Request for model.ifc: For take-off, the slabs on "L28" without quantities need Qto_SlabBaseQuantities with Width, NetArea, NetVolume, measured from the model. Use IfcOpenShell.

First a look at what the model holds.

```python
import ifcopenshell
import ifcopenshell.util.element
import ifcopenshell.util.unit

model = ifcopenshell.open("model.ifc")
print(model.schema)
for unit_type in ("LENGTHUNIT", "AREAUNIT", "VOLUMEUNIT"):
    print(unit_type, ifcopenshell.util.unit.calculate_unit_scale(model, unit_type))
storey = next(s for s in model.by_type("IfcBuildingStorey") if s.Name == "L28")
slabs = [e for e in ifcopenshell.util.element.get_decomposition(storey) if e.is_a("IfcSlab")]
for e in sorted(slabs, key=lambda e: e.id()):
    print(e.id(), e.is_a(), e.Name, list(ifcopenshell.util.element.get_psets(e, qtos_only=True)), sep=" | ")
```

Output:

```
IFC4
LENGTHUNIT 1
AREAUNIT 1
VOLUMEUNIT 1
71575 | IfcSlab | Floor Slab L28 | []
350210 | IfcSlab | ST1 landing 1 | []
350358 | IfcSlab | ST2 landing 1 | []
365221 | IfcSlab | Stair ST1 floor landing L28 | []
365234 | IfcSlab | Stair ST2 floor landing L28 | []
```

```python
import ifcopenshell
import ifcopenshell.api.pset
import ifcopenshell.geom
import ifcopenshell.util.element
import ifcopenshell.util.shape
import ifcopenshell.util.unit

model = ifcopenshell.open("model.ifc")
unit_scale = ifcopenshell.util.unit.calculate_unit_scale(model)
area_scale = ifcopenshell.util.unit.calculate_unit_scale(model, "AREAUNIT")
volume_scale = ifcopenshell.util.unit.calculate_unit_scale(model, "VOLUMEUNIT")
settings = ifcopenshell.geom.settings()

storey = next(s for s in model.by_type("IfcBuildingStorey") if s.Name == "L28")
slabs = [e for e in ifcopenshell.util.element.get_decomposition(storey) if e.is_a("IfcSlab")]

for e in sorted(slabs, key=lambda e: e.id()):
    if ifcopenshell.util.element.get_psets(e, qtos_only=True, should_inherit=False):
        continue
    # Geometry comes back in metres, in the element's own axes.
    shape = ifcopenshell.geom.create_shape(settings, e)
    values = {
        "Width": ifcopenshell.util.shape.get_z(shape.geometry) / unit_scale,
        "NetArea": ifcopenshell.util.shape.get_footprint_area(shape.geometry) / area_scale,
        "NetVolume": ifcopenshell.util.shape.get_volume(shape.geometry) / volume_scale,
    }
    qto = ifcopenshell.api.pset.add_qto(model, product=e, name="Qto_SlabBaseQuantities")
    ifcopenshell.api.pset.edit_qto(model, qto=qto, properties=values)
    print(e.id(), {k: round(v, 3) for k, v in values.items()})

model.write("model_updated.ifc")
```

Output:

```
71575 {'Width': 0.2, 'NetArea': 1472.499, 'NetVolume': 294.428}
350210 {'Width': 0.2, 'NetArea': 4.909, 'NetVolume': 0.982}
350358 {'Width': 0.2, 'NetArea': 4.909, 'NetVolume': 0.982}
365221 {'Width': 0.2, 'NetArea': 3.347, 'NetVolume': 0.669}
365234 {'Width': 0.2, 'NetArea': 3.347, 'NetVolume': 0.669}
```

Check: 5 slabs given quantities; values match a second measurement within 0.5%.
